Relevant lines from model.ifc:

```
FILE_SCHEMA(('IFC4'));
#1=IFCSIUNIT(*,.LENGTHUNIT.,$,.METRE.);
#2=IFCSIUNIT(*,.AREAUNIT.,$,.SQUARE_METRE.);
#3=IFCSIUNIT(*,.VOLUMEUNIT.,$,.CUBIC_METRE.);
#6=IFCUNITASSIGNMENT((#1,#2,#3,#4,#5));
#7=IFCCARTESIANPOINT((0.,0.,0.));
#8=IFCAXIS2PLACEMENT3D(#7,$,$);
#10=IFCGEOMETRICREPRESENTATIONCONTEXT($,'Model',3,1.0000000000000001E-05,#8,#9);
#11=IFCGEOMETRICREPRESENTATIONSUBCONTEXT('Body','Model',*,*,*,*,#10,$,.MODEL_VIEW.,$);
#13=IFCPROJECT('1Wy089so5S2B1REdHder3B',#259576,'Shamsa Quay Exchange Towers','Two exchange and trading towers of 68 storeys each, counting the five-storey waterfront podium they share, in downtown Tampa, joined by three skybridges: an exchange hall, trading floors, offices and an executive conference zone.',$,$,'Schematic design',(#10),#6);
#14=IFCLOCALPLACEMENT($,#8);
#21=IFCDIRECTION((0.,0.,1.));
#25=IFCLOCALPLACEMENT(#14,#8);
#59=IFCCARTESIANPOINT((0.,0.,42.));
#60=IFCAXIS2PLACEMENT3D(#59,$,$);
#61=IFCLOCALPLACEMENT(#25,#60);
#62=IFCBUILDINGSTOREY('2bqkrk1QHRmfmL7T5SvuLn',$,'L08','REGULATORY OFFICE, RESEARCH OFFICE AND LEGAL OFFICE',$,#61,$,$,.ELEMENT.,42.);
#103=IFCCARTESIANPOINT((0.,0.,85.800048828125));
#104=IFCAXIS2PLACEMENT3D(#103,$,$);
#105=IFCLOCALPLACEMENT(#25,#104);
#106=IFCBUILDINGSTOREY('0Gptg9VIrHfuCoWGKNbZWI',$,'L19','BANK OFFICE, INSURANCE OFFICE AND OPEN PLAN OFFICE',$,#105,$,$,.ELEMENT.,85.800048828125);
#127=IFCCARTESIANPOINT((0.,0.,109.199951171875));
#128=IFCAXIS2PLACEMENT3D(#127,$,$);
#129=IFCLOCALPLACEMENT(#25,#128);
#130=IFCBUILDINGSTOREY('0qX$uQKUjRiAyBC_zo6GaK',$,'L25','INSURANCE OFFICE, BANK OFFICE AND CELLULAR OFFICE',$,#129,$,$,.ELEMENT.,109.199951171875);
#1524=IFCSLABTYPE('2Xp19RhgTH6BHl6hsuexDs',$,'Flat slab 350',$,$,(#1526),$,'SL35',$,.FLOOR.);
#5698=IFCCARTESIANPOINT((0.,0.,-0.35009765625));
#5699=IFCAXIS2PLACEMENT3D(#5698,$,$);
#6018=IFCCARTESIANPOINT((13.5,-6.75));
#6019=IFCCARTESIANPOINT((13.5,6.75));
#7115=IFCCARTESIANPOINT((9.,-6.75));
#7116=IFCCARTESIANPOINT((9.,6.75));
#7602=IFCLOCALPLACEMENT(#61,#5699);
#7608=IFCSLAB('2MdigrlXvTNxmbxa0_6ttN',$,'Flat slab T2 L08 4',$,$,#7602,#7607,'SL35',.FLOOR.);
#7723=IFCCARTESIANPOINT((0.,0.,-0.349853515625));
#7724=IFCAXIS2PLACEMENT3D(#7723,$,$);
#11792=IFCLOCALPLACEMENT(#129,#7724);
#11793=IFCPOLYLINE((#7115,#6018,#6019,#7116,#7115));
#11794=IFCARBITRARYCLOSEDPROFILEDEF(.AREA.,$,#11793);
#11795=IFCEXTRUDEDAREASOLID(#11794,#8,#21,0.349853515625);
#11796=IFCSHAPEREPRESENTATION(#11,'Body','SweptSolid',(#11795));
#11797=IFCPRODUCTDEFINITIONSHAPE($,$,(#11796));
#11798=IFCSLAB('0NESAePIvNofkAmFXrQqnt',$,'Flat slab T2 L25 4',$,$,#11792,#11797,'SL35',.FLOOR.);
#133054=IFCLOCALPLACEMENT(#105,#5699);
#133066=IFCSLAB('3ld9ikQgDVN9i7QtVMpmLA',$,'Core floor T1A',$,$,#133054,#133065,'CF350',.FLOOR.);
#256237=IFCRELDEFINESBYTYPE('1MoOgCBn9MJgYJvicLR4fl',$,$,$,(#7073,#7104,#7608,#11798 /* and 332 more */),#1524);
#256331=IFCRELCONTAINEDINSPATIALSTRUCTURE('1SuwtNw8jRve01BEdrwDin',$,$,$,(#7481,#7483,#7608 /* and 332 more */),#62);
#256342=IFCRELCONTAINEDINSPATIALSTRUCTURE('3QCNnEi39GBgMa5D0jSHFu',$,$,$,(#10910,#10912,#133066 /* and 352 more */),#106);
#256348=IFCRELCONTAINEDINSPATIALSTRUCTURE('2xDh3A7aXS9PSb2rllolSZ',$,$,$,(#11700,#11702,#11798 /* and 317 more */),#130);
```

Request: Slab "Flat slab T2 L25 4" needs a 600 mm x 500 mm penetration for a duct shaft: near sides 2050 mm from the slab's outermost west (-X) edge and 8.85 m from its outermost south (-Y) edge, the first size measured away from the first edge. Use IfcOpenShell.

```python
import numpy as np
import ifcopenshell
import ifcopenshell.api.feature
import ifcopenshell.api.geometry
import ifcopenshell.api.root
import ifcopenshell.geom
import ifcopenshell.util.placement
import ifcopenshell.util.representation
import ifcopenshell.util.shape
import ifcopenshell.util.unit

model = ifcopenshell.open("model.ifc")
unit_scale = ifcopenshell.util.unit.calculate_unit_scale(model)
settings = ifcopenshell.geom.settings()


def volume(element):
    """Net volume in cubic metres, openings subtracted."""
    shape = ifcopenshell.geom.create_shape(settings, element)
    return ifcopenshell.util.shape.get_volume(shape.geometry)


slab = model.by_guid("0NESAePIvNofkAmFXrQqnt")
before = volume(slab)

# Extent in the slab's own axes, in metres. The edges named are its -X and -Y sides.
slab_shape = ifcopenshell.geom.create_shape(settings, slab)
vertices = ifcopenshell.util.shape.get_vertices(slab_shape.geometry)
x_min, y_min, bottom = vertices.min(axis=0)
top = vertices[:, 2].max()

opening = ifcopenshell.api.root.create_entity(model, ifc_class="IfcOpeningElement", name="Duct shaft opening", predefined_type="OPENING")
context = ifcopenshell.util.representation.get_context(model, "Model", "Body", "MODEL_VIEW")
width, depth = 0.6, 0.5
outline = [(0.0, 0.0), (width, 0.0), (width, depth), (0.0, depth), (0.0, 0.0)]
# Overshoot both faces by 50 mm so the cut is clean.
shape = ifcopenshell.api.geometry.add_slab_representation(
    model, context=context, depth=top - bottom + 0.1, polyline=outline
)
ifcopenshell.api.geometry.assign_representation(model, product=opening, representation=shape)

matrix = ifcopenshell.util.placement.get_local_placement(slab.ObjectPlacement)
matrix[:, 3] = matrix @ np.append(np.array([x_min + 2.05, y_min + 8.85, bottom - 0.05]) / unit_scale, 1.0)
ifcopenshell.api.geometry.edit_object_placement(model, product=opening, matrix=matrix, is_si=False)
ifcopenshell.api.feature.add_feature(model, feature=opening, element=slab)

after = volume(slab)

print(f"slab volume {before:.3f} -> {after:.3f} m3")

model.write("model_updated.ifc")
```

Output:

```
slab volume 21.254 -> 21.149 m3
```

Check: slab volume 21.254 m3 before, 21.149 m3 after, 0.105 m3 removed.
